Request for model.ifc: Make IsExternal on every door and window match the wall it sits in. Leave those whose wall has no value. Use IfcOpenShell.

First a look at what the model holds.

```python
import ifcopenshell
import ifcopenshell.util.element

model = ifcopenshell.open("model.ifc")
print(model.schema)
seen = {}
for e in model.by_type("IfcDoor") + model.by_type("IfcWindow"):
    if not e.FillsVoids:
        continue
    host = e.FillsVoids[0].RelatingOpeningElement.VoidsElements[0].RelatingBuildingElement
    own = ifcopenshell.util.element.get_pset(e, f"Pset_{e.is_a()[3:].removesuffix('StandardCase')}Common", "IsExternal")
    wall = ifcopenshell.util.element.get_pset(host, "Pset_WallCommon", "IsExternal")
    seen[e.is_a(), own, wall] = seen.get((e.is_a(), own, wall), 0) + 1
for (cls, own, wall), count in sorted(seen.items(), key=str):
    print(count, cls, "IsExternal:", own, "| host wall:", wall)
```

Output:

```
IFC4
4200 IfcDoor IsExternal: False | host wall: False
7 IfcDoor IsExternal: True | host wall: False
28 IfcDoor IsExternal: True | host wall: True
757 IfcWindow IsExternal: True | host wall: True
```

```python
import ifcopenshell
import ifcopenshell.api.pset
import ifcopenshell.util.element

model = ifcopenshell.open("model.ifc")

count = 0
for ifc_class, pset_name in (("IfcDoor", "Pset_DoorCommon"), ("IfcWindow", "Pset_WindowCommon")):
    for e in model.by_type(ifc_class):
        if not e.FillsVoids:
            continue
        host = e.FillsVoids[0].RelatingOpeningElement.VoidsElements[0].RelatingBuildingElement
        external = ifcopenshell.util.element.get_pset(host, "Pset_WallCommon", "IsExternal")
        if external is None or ifcopenshell.util.element.get_pset(e, pset_name, "IsExternal") == external:
            continue
        found = ifcopenshell.util.element.get_pset(e, pset_name, should_inherit=False)
        if found:
            pset = model.by_id(found["id"])
            if len(ifcopenshell.util.element.get_elements_by_pset(pset)) > 1:
                pset = ifcopenshell.api.pset.unshare_pset(model, products=[e], pset=pset)[0]
        else:
            pset = ifcopenshell.api.pset.add_pset(model, product=e, name=pset_name)
        ifcopenshell.api.pset.edit_pset(model, pset=pset, properties={"IsExternal": external})
        count += 1

print(count, "updated")

model.write("model_rev.ifc")
```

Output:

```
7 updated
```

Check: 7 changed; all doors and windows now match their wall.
